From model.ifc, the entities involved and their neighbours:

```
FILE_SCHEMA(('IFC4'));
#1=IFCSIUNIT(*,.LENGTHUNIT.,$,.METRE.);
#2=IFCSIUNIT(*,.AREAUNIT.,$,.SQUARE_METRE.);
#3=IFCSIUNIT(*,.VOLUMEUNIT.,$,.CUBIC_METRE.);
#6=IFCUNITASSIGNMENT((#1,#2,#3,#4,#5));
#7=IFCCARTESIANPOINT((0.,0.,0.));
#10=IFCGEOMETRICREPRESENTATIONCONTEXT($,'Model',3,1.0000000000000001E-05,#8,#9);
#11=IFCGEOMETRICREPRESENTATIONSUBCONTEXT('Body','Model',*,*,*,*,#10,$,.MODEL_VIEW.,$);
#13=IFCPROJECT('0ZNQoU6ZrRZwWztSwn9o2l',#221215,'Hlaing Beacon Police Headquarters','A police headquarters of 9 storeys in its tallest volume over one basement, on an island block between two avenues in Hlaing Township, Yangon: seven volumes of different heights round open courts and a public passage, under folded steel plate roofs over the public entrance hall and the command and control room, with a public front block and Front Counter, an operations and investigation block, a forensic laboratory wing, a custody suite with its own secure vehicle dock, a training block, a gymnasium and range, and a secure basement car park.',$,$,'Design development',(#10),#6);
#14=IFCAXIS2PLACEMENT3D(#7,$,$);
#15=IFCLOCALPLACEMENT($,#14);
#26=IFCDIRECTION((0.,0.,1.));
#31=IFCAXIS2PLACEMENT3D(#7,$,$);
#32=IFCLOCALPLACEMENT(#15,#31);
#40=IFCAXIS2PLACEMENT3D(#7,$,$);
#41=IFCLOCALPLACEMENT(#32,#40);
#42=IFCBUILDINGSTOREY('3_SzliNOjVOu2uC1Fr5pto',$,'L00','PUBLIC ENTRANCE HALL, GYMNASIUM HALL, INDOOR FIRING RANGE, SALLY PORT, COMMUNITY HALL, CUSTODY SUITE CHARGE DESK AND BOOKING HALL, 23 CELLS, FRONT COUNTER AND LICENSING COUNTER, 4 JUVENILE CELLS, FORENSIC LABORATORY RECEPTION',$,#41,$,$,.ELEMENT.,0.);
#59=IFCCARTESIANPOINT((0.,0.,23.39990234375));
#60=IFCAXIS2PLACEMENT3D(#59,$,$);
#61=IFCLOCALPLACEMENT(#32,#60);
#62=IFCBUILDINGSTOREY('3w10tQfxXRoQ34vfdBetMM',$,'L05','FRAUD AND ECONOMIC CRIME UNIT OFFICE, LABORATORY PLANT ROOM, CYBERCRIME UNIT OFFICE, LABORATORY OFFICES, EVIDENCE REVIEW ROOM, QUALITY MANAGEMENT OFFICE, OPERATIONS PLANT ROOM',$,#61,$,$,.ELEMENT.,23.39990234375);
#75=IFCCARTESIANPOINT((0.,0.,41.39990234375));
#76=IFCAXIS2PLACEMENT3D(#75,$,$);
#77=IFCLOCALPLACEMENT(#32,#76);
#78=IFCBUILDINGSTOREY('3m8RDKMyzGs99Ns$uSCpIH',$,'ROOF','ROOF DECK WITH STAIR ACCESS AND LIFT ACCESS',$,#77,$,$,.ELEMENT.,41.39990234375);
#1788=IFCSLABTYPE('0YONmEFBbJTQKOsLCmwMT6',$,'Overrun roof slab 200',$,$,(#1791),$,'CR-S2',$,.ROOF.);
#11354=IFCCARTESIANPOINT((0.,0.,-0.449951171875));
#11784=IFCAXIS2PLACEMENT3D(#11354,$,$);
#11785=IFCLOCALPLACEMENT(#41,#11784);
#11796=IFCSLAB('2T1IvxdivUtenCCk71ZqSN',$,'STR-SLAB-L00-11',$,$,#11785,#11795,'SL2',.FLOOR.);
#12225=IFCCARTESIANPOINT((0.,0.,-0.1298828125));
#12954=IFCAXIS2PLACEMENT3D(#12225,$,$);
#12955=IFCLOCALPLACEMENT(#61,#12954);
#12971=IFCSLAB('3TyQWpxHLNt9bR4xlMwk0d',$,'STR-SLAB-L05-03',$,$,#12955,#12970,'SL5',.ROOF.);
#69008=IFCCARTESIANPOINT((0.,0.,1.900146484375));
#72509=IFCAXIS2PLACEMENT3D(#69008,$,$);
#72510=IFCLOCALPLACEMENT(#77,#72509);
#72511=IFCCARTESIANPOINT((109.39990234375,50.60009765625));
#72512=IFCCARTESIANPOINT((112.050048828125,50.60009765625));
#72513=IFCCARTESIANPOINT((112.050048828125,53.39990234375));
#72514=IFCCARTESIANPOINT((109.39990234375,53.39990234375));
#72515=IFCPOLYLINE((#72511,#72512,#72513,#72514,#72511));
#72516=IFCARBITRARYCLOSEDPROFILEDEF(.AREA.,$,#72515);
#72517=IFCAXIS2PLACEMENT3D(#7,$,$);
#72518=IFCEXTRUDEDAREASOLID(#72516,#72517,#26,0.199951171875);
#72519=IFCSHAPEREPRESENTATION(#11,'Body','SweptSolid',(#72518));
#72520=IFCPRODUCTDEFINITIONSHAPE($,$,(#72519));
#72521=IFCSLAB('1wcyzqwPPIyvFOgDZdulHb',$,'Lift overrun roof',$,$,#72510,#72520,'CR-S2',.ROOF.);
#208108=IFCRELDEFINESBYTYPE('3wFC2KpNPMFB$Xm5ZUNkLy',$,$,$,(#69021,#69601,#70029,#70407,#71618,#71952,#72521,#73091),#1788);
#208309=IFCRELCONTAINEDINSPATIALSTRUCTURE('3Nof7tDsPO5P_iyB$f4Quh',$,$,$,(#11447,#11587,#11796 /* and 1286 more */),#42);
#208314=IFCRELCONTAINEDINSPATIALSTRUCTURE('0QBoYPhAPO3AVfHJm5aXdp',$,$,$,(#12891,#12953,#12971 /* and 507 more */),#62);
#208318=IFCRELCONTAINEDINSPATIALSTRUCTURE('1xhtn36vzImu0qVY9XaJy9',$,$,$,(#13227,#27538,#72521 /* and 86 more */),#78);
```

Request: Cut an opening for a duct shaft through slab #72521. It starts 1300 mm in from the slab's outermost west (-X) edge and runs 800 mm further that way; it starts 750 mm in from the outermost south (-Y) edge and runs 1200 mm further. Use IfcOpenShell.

```python
import numpy as np
import ifcopenshell
import ifcopenshell.api.feature
import ifcopenshell.api.geometry
import ifcopenshell.api.root
import ifcopenshell.geom
import ifcopenshell.util.placement
import ifcopenshell.util.representation
import ifcopenshell.util.shape
import ifcopenshell.util.unit

model = ifcopenshell.open("model.ifc")
unit_scale = ifcopenshell.util.unit.calculate_unit_scale(model)
settings = ifcopenshell.geom.settings()


def volume(element):
    """Net volume in cubic metres, openings subtracted."""
    shape = ifcopenshell.geom.create_shape(settings, element)
    return ifcopenshell.util.shape.get_volume(shape.geometry)


slab = model.by_guid("1wcyzqwPPIyvFOgDZdulHb")
before = volume(slab)

# Extent in the slab's own axes, in metres. The edges named are its -X and -Y sides.
slab_shape = ifcopenshell.geom.create_shape(settings, slab)
vertices = ifcopenshell.util.shape.get_vertices(slab_shape.geometry)
x_min, y_min, bottom = vertices.min(axis=0)
top = vertices[:, 2].max()

opening = ifcopenshell.api.root.create_entity(model, ifc_class="IfcOpeningElement", name="Duct shaft opening", predefined_type="OPENING")
context = ifcopenshell.util.representation.get_context(model, "Model", "Body", "MODEL_VIEW")
width, depth = 0.8, 1.2
outline = [(0.0, 0.0), (width, 0.0), (width, depth), (0.0, depth), (0.0, 0.0)]
# Overshoot both faces by 50 mm so the cut is clean.
shape = ifcopenshell.api.geometry.add_slab_representation(
    model, context=context, depth=top - bottom + 0.1, polyline=outline
)
ifcopenshell.api.geometry.assign_representation(model, product=opening, representation=shape)

matrix = ifcopenshell.util.placement.get_local_placement(slab.ObjectPlacement)
matrix[:, 3] = matrix @ np.append(np.array([x_min + 1.3, y_min + 0.75, bottom - 0.05]) / unit_scale, 1.0)
ifcopenshell.api.geometry.edit_object_placement(model, product=opening, matrix=matrix, is_si=False)
ifcopenshell.api.feature.add_feature(model, feature=opening, element=slab)

after = volume(slab)

print(f"slab volume {before:.3f} -> {after:.3f} m3")

model.write("model_updated.ifc")
```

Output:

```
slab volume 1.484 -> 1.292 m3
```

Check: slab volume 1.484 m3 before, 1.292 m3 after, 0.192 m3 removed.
